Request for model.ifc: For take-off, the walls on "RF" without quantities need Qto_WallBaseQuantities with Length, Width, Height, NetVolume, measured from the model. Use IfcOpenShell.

First a look at what the model holds.

```python
import ifcopenshell
import ifcopenshell.util.element
import ifcopenshell.util.unit

model = ifcopenshell.open("model.ifc")
print(model.schema)
for unit_type in ("LENGTHUNIT", "AREAUNIT", "VOLUMEUNIT"):
    print(unit_type, ifcopenshell.util.unit.calculate_unit_scale(model, unit_type))
storey = next(s for s in model.by_type("IfcBuildingStorey") if s.Name == "RF")
walls = [e for e in ifcopenshell.util.element.get_decomposition(storey) if e.is_a("IfcWall")]
for e in sorted(walls, key=lambda e: e.id()):
    print(e.id(), e.is_a(), e.Name, list(ifcopenshell.util.element.get_psets(e, qtos_only=True)), sep=" | ")
```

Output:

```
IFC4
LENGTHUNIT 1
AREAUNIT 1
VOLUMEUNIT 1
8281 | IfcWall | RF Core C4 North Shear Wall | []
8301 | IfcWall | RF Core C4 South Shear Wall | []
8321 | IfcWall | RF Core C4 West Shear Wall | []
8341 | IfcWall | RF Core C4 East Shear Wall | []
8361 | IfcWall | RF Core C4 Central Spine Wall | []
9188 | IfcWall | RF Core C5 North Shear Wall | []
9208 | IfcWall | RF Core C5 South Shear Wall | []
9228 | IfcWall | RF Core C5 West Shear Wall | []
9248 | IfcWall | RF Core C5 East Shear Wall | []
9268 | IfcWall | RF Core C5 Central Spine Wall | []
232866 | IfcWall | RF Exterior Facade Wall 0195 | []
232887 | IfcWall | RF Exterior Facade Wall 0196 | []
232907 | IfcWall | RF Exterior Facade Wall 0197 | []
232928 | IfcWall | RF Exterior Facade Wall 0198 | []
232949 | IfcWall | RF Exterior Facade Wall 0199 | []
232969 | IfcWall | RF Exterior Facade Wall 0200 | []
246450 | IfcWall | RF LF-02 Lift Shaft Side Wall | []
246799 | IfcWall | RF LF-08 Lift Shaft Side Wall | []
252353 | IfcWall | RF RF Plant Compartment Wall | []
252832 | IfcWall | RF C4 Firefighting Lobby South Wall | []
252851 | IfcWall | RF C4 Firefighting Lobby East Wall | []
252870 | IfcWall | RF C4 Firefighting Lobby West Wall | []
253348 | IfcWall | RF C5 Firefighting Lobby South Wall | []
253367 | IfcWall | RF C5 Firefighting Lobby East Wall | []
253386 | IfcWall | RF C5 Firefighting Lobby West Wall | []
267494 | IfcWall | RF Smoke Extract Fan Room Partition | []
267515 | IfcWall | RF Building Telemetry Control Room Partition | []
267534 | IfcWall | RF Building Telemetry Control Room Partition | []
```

```python
import ifcopenshell
import ifcopenshell.api.pset
import ifcopenshell.geom
import ifcopenshell.util.element
import ifcopenshell.util.shape
import ifcopenshell.util.unit

model = ifcopenshell.open("model.ifc")
unit_scale = ifcopenshell.util.unit.calculate_unit_scale(model)
volume_scale = ifcopenshell.util.unit.calculate_unit_scale(model, "VOLUMEUNIT")
settings = ifcopenshell.geom.settings()

storey = next(s for s in model.by_type("IfcBuildingStorey") if s.Name == "RF")
walls = [e for e in ifcopenshell.util.element.get_decomposition(storey) if e.is_a("IfcWall")]

for e in sorted(walls, key=lambda e: e.id()):
    if ifcopenshell.util.element.get_psets(e, qtos_only=True, should_inherit=False):
        continue
    # Geometry comes back in metres, in the element's own axes.
    shape = ifcopenshell.geom.create_shape(settings, e)
    values = {
        "Length": ifcopenshell.util.shape.get_x(shape.geometry) / unit_scale,
        "Width": ifcopenshell.util.shape.get_y(shape.geometry) / unit_scale,
        "Height": ifcopenshell.util.shape.get_z(shape.geometry) / unit_scale,
        "NetVolume": ifcopenshell.util.shape.get_volume(shape.geometry) / volume_scale,
    }
    qto = ifcopenshell.api.pset.add_qto(model, product=e, name="Qto_WallBaseQuantities")
    ifcopenshell.api.pset.edit_qto(model, qto=qto, properties=values)
    print(e.id(), {k: round(v, 3) for k, v in values.items()})

model.write("model_updated.ifc")
```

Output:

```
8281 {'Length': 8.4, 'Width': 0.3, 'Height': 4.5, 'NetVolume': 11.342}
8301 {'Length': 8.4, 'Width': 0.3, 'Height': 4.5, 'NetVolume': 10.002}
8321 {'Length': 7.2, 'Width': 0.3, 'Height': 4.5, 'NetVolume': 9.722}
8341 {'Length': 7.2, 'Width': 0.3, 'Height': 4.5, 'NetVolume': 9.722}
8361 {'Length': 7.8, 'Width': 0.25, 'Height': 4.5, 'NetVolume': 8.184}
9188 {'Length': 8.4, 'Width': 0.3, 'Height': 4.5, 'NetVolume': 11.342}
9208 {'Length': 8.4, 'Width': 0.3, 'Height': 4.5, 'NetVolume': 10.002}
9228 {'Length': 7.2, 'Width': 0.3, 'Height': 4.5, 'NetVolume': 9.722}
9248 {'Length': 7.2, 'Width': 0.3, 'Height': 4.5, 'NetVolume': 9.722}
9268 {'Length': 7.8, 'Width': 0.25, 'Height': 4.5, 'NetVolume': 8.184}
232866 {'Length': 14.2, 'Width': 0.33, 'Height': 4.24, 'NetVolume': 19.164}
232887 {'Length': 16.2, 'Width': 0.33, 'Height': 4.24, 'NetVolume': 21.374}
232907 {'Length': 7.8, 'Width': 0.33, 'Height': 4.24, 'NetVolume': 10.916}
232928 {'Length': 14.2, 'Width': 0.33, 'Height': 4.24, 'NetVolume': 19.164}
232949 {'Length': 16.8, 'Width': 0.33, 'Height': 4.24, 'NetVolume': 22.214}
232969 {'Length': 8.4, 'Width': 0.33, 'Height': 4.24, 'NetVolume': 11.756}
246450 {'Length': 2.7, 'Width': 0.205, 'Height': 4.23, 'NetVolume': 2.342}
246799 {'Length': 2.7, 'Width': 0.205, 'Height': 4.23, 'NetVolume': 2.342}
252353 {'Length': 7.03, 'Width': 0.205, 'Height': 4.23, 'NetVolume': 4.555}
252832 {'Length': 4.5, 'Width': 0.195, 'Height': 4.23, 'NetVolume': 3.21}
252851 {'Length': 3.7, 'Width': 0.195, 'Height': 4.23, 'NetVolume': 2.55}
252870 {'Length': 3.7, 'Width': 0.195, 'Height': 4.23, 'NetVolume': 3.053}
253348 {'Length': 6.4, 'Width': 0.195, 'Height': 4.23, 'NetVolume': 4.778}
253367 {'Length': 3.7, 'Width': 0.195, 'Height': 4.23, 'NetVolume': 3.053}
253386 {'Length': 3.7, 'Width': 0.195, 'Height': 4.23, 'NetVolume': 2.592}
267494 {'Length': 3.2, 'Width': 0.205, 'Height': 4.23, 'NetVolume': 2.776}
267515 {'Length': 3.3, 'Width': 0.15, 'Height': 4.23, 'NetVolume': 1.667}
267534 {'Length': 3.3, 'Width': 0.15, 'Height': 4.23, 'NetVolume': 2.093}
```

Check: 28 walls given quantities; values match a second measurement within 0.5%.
